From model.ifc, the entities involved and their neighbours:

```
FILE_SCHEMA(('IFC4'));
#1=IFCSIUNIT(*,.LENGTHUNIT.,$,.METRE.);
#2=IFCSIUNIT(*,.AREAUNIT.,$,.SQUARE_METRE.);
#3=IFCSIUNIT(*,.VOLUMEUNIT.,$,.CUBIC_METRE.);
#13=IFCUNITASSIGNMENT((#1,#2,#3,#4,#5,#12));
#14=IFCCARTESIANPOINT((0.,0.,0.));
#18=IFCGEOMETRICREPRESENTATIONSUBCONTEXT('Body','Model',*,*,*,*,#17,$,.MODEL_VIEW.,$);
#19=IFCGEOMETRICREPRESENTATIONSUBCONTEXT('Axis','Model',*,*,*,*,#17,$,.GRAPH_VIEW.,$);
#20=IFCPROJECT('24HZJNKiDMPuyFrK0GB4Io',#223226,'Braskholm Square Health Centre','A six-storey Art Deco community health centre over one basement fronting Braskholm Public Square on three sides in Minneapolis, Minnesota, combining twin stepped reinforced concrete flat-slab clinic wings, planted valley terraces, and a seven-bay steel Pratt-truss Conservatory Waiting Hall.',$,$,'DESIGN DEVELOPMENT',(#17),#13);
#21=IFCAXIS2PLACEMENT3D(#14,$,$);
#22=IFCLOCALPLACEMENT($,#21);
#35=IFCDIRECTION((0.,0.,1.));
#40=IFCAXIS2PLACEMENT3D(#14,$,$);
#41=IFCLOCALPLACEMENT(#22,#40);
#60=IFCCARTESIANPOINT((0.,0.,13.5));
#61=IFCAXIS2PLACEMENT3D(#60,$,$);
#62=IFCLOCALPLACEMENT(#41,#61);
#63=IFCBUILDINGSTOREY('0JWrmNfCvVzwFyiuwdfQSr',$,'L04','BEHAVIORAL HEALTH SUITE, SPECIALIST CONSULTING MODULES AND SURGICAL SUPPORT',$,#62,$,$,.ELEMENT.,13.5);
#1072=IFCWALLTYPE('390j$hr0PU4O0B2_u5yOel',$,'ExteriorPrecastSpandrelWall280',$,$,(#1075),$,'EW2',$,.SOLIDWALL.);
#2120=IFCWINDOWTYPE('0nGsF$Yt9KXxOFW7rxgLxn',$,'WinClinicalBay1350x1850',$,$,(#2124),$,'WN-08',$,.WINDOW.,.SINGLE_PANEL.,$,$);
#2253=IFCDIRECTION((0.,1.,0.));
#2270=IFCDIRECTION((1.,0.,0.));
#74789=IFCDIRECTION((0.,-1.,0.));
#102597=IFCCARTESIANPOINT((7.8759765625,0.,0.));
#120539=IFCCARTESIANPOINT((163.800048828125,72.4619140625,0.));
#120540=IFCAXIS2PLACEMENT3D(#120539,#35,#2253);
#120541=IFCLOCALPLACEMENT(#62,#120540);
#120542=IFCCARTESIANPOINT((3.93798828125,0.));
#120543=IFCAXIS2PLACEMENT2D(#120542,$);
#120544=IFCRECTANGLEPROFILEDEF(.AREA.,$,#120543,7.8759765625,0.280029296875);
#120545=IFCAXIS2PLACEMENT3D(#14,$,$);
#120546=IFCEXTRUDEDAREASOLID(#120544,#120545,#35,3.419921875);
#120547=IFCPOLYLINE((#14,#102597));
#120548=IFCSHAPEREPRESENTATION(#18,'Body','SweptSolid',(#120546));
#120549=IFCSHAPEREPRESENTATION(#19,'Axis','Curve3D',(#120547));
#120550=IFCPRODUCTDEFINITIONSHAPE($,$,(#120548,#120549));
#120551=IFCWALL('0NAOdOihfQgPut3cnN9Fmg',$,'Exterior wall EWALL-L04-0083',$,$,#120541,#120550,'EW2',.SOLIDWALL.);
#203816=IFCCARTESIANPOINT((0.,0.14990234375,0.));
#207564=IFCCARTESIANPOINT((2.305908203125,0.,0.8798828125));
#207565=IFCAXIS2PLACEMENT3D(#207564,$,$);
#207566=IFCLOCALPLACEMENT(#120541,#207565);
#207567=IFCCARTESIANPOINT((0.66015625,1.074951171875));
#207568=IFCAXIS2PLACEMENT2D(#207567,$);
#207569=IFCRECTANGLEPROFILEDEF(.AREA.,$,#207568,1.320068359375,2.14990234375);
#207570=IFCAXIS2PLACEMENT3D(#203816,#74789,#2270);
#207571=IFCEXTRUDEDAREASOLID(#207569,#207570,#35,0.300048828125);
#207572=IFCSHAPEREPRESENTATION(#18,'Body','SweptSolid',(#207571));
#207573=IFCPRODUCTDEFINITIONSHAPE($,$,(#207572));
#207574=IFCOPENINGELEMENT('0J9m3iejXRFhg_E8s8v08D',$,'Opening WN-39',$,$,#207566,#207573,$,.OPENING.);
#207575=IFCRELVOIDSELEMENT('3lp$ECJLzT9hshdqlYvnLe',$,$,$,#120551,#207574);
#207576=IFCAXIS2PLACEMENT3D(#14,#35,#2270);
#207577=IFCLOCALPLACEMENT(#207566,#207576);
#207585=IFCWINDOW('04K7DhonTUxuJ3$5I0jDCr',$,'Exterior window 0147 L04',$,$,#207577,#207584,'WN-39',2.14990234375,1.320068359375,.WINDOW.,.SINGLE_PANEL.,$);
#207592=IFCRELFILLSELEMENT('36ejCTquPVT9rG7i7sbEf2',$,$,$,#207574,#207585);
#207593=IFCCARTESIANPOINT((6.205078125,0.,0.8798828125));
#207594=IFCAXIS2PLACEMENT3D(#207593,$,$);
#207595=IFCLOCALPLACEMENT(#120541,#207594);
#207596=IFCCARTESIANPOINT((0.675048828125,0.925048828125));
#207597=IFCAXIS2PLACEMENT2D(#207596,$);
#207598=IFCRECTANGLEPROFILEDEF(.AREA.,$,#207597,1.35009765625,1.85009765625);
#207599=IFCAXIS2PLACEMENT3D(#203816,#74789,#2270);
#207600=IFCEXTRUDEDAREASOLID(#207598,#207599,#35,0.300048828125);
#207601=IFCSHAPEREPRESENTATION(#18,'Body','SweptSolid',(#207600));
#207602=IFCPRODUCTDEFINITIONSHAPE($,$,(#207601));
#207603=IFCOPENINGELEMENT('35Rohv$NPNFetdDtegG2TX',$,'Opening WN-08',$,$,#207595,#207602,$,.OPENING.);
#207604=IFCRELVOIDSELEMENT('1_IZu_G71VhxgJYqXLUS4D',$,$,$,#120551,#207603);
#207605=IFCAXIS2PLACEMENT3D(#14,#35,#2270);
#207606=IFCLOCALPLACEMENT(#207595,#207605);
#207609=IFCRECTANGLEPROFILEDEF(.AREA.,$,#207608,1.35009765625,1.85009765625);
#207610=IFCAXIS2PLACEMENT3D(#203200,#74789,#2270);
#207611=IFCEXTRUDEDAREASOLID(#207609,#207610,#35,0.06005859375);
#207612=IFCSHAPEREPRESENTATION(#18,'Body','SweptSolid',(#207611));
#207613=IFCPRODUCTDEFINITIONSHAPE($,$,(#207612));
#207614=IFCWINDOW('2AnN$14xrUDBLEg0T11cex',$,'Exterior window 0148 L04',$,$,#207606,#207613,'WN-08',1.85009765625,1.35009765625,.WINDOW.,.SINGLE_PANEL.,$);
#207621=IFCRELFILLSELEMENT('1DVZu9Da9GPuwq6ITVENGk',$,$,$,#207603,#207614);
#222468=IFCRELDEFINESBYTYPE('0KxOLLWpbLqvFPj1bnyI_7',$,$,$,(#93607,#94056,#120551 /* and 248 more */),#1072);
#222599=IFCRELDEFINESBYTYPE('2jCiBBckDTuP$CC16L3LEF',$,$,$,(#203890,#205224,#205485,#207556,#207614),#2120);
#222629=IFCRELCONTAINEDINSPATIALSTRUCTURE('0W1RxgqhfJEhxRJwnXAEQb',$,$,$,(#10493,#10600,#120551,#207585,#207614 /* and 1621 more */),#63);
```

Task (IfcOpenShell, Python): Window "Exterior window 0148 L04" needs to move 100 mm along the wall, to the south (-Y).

```python
import ifcopenshell
import ifcopenshell.api.geometry
import ifcopenshell.util.placement

model = ifcopenshell.open("model.ifc")

window = model.by_guid("2AnN$14xrUDBLEg0T11cex")
opening = window.FillsVoids[0].RelatingOpeningElement
wall = opening.VoidsElements[0].RelatingBuildingElement

wall_matrix = ifcopenshell.util.placement.get_local_placement(wall.ObjectPlacement)
shift = wall_matrix[:3, 0] * -0.1
before = ifcopenshell.util.placement.get_local_placement(window.ObjectPlacement)[:3, 3].copy()

# The window is placed relative to its opening, so it follows when the opening moves.
matrix = ifcopenshell.util.placement.get_local_placement(opening.ObjectPlacement)
matrix[:3, 3] += shift
ifcopenshell.api.geometry.edit_object_placement(
    model, product=opening, matrix=matrix, is_si=False, should_transform_children=True
)

after = ifcopenshell.util.placement.get_local_placement(window.ObjectPlacement)[:3, 3]
print("window moved by", (after - before).round(3) + 0.0)

model.write("model_edited.ifc")
```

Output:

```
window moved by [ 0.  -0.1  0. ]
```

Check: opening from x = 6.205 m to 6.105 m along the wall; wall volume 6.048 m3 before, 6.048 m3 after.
